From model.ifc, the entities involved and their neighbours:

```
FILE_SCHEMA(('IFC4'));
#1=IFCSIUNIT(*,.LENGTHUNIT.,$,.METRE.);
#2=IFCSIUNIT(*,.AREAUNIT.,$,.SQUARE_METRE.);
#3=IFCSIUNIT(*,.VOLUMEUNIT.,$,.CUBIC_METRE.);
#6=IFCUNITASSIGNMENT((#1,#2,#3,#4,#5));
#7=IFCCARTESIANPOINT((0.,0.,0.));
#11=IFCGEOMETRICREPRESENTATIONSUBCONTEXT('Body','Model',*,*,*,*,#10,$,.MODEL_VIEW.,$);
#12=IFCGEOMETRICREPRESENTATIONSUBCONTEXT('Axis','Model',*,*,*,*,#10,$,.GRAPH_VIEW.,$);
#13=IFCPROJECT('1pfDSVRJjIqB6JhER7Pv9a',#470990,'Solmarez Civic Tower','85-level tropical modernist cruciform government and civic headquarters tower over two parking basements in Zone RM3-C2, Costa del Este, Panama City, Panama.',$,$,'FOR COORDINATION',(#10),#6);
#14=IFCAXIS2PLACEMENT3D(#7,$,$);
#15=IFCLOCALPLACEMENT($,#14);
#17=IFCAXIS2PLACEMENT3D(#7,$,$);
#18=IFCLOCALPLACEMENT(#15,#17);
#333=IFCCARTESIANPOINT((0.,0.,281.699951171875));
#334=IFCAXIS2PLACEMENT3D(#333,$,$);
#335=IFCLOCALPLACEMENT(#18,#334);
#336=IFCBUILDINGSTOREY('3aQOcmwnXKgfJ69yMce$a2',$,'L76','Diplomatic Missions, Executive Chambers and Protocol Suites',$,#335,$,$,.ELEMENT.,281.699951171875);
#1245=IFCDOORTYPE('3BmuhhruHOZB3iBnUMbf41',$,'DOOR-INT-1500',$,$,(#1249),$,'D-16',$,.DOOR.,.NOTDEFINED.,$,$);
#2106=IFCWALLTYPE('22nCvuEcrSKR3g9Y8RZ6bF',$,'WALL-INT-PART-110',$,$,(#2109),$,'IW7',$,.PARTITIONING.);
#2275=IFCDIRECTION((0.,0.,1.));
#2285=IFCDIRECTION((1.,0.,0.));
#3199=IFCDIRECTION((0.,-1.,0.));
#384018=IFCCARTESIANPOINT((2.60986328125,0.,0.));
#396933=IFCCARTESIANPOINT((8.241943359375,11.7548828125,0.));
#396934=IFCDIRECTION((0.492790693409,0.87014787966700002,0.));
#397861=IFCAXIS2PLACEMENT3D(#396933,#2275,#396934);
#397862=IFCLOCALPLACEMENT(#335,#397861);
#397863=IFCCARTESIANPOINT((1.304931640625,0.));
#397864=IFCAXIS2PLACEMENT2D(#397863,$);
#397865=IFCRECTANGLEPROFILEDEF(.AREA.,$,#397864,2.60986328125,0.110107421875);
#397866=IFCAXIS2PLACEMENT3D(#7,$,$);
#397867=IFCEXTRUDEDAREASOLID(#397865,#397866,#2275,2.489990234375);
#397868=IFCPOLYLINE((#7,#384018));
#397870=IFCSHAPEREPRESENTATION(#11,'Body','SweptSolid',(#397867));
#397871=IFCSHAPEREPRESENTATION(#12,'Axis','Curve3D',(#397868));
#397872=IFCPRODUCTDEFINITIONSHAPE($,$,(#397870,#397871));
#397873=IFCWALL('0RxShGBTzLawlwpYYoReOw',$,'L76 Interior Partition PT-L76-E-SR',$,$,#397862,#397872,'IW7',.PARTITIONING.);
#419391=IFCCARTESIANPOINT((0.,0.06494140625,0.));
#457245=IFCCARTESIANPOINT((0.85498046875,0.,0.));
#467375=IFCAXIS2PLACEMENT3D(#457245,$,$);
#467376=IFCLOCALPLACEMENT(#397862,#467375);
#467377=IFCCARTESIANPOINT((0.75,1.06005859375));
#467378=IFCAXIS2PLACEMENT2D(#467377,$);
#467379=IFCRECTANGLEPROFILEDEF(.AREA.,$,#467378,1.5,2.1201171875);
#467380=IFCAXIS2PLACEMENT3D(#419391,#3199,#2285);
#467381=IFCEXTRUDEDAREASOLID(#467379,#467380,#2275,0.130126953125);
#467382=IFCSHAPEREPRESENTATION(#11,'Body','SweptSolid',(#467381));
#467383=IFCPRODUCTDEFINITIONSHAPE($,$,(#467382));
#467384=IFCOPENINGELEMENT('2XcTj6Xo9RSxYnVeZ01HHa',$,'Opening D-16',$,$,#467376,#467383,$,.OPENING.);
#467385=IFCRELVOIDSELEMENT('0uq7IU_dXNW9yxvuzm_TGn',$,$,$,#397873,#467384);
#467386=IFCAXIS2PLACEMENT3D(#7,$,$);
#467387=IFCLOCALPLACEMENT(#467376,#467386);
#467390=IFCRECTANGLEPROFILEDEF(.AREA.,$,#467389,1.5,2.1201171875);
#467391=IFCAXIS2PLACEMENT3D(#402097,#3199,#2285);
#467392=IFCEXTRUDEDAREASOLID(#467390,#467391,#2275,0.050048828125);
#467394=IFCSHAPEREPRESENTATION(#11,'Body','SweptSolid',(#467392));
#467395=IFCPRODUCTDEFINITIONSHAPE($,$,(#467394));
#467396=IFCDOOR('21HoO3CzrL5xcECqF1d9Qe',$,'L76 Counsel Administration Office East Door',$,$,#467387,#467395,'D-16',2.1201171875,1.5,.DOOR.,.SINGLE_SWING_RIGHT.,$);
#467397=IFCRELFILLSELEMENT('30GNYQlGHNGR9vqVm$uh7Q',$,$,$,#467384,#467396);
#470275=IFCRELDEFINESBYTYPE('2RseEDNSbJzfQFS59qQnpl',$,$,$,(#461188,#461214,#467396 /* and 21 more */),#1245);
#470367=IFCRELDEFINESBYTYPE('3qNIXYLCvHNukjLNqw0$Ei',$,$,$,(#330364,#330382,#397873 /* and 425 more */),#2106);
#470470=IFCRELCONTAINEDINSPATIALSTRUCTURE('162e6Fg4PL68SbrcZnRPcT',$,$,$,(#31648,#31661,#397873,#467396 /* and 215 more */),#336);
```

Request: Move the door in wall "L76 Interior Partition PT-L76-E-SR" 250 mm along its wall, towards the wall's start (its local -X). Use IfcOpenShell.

```python
import ifcopenshell
import ifcopenshell.api.geometry
import ifcopenshell.util.placement
import ifcopenshell.util.unit

model = ifcopenshell.open("model.ifc")
unit_scale = ifcopenshell.util.unit.calculate_unit_scale(model)

door = model.by_id(467396)
opening = door.FillsVoids[0].RelatingOpeningElement
wall = opening.VoidsElements[0].RelatingBuildingElement

wall_matrix = ifcopenshell.util.placement.get_local_placement(wall.ObjectPlacement)
shift = wall_matrix[:3, 0] * -0.25 / unit_scale
before = ifcopenshell.util.placement.get_local_placement(door.ObjectPlacement)[:3, 3].copy()

# The door is placed relative to its opening, so it follows when the opening moves.
matrix = ifcopenshell.util.placement.get_local_placement(opening.ObjectPlacement)
matrix[:3, 3] += shift
ifcopenshell.api.geometry.edit_object_placement(
    model, product=opening, matrix=matrix, is_si=False, should_transform_children=True
)

after = ifcopenshell.util.placement.get_local_placement(door.ObjectPlacement)[:3, 3]
print("door moved by", (after - before).round(3) + 0.0)

model.write("model_updated.ifc")
```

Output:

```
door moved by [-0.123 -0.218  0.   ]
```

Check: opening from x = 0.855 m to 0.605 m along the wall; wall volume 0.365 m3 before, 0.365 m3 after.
